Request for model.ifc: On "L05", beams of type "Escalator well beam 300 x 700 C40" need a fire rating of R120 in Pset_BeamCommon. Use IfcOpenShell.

First a look at what the model holds.

```python
import ifcopenshell
import ifcopenshell.util.element

model = ifcopenshell.open("model.ifc")
print(model.schema)
storey = next(s for s in model.by_type("IfcBuildingStorey") if s.Name == "L05")
beams = [e for e in ifcopenshell.util.element.get_decomposition(storey) if e.is_a("IfcBeam")]
seen = {}
for e in beams:
    element_type = ifcopenshell.util.element.get_type(e)
    key = (element_type.Name if element_type != e and element_type else None, ifcopenshell.util.element.get_pset(e, "Pset_BeamCommon", "FireRating"))
    seen[key] = seen.get(key, 0) + 1
for (name, value), count in sorted(seen.items(), key=str):
    print(count, "x", name, "|", value)
```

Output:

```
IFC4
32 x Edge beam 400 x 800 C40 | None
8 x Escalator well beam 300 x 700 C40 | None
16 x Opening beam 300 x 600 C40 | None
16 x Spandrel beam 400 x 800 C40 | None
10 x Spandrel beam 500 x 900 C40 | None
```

```python
import ifcopenshell
import ifcopenshell.api.pset
import ifcopenshell.util.element

model = ifcopenshell.open("model.ifc")

storey = next(s for s in model.by_type("IfcBuildingStorey") if s.Name == "L05")
beams = [e for e in ifcopenshell.util.element.get_decomposition(storey) if e.is_a("IfcBeam")]

count = 0
for e in beams:
    element_type = ifcopenshell.util.element.get_type(e)
    if element_type in (None, e) or element_type.Name != "Escalator well beam 300 x 700 C40":
        continue
    # add_pset returns the element's existing set when there is one.
    pset = ifcopenshell.api.pset.add_pset(model, product=e, name="Pset_BeamCommon")
    ifcopenshell.api.pset.edit_pset(model, pset=pset, properties={"FireRating": "R120"})
    count += 1

print(count, "beams updated")

model.write("model_updated.ifc")
```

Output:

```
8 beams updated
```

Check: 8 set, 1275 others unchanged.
